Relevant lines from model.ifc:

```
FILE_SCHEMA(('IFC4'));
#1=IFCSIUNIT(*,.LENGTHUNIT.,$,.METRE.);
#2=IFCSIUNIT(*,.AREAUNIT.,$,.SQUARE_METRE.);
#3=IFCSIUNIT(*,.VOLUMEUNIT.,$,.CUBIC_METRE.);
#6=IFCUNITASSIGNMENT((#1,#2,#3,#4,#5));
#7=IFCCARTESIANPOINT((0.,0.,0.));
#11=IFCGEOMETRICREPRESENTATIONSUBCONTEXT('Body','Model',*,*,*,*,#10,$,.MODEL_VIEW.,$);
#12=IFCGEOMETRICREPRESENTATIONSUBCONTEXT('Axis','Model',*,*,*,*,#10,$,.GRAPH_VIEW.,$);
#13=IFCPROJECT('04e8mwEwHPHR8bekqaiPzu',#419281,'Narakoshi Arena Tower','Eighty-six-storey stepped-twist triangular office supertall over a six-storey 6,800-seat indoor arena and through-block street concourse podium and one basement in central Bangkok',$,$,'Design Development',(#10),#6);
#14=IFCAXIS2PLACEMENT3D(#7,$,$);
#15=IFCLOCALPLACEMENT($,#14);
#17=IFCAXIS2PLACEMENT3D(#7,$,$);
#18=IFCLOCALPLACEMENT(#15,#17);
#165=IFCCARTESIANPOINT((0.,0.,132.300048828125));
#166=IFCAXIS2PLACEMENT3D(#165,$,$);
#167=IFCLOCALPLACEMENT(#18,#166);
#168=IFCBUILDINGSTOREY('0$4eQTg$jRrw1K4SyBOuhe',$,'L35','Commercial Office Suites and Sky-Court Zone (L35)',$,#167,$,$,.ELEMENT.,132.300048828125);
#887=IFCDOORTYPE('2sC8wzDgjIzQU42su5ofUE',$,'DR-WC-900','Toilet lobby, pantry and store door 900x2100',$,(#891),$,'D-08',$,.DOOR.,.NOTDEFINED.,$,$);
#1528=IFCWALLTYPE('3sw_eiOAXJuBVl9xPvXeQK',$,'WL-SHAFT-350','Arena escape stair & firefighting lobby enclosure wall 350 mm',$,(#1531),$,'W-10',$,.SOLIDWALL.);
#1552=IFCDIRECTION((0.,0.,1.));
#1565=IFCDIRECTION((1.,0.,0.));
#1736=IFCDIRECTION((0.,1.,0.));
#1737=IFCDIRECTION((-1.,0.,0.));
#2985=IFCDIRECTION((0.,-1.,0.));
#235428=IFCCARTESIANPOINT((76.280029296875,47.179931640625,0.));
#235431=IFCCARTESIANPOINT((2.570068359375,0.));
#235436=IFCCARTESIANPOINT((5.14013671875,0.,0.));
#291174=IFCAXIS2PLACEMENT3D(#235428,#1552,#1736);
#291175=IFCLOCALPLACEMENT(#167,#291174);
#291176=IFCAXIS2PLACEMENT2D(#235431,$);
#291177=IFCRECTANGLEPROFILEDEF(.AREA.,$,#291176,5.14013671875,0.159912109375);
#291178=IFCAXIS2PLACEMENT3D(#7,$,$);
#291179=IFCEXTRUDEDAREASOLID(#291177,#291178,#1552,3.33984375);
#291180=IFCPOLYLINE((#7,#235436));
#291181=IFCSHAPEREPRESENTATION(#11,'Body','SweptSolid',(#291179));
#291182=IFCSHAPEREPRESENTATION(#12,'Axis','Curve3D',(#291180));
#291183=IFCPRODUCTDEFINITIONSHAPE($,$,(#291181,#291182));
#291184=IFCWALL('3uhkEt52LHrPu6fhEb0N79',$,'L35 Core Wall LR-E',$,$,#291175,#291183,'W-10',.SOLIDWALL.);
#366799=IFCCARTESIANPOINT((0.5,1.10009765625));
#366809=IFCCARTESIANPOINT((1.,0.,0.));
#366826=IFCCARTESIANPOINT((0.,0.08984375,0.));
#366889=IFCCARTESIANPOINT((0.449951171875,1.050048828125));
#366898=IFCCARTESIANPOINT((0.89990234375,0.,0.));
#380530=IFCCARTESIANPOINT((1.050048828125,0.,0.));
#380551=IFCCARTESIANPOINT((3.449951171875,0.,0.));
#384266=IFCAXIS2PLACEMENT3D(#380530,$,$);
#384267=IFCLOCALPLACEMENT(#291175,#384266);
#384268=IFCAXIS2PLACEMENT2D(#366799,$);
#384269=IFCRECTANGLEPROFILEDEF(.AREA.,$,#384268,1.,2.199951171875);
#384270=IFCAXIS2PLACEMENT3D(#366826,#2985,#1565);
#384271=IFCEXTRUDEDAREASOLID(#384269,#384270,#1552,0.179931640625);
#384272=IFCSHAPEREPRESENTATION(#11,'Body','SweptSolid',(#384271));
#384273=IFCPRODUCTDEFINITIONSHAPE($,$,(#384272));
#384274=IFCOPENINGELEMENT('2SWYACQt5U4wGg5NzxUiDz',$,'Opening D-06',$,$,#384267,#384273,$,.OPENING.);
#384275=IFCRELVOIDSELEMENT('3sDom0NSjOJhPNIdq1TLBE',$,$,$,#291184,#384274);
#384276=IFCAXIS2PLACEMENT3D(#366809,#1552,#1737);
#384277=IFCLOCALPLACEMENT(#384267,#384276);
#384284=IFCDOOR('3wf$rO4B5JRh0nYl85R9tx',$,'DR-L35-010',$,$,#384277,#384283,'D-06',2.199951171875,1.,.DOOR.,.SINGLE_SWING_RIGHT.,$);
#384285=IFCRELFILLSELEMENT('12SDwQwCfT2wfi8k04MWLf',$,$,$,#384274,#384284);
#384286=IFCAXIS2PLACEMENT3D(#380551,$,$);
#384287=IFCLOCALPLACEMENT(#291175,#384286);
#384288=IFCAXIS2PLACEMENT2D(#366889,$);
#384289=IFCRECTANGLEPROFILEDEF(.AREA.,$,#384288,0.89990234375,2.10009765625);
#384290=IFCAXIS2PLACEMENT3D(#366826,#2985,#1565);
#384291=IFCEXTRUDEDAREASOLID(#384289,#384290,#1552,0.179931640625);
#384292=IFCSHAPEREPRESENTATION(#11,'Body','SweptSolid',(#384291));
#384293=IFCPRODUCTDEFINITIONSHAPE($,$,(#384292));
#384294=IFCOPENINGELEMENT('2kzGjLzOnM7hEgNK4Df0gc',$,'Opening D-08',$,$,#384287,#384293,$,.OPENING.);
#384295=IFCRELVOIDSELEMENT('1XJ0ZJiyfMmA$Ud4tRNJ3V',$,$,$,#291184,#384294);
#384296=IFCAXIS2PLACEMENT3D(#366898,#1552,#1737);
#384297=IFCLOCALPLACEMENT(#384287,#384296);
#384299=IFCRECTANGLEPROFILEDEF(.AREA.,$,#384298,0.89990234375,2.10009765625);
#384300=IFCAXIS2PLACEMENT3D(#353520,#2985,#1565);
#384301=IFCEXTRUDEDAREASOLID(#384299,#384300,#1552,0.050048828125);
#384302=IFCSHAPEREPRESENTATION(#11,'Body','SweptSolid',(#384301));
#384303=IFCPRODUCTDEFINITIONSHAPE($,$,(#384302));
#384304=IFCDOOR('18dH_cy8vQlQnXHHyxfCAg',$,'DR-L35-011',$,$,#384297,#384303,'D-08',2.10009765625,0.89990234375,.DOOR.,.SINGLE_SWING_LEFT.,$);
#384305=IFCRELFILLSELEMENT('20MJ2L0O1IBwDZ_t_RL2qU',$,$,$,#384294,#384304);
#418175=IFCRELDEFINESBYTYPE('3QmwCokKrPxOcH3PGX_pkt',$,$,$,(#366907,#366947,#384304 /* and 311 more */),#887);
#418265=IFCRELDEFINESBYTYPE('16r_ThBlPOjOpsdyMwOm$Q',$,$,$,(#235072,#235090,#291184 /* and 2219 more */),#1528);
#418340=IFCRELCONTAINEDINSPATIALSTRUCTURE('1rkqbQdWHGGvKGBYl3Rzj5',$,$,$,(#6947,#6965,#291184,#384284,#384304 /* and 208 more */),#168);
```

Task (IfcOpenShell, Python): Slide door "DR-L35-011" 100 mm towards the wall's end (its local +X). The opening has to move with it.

```python
import ifcopenshell
import ifcopenshell.api.geometry
import ifcopenshell.util.placement
import ifcopenshell.util.unit

model = ifcopenshell.open("model.ifc")
unit_scale = ifcopenshell.util.unit.calculate_unit_scale(model)

door = model.by_guid("18dH_cy8vQlQnXHHyxfCAg")
opening = door.FillsVoids[0].RelatingOpeningElement
wall = opening.VoidsElements[0].RelatingBuildingElement

wall_matrix = ifcopenshell.util.placement.get_local_placement(wall.ObjectPlacement)
shift = wall_matrix[:3, 0] * 0.1 / unit_scale
before = ifcopenshell.util.placement.get_local_placement(door.ObjectPlacement)[:3, 3].copy()

# The door is placed relative to its opening, so it follows when the opening moves.
matrix = ifcopenshell.util.placement.get_local_placement(opening.ObjectPlacement)
matrix[:3, 3] += shift
ifcopenshell.api.geometry.edit_object_placement(
    model, product=opening, matrix=matrix, is_si=False, should_transform_children=True
)

after = ifcopenshell.util.placement.get_local_placement(door.ObjectPlacement)[:3, 3]
print("door moved by", (after - before).round(3) + 0.0)

model.write("model_edited.ifc")
```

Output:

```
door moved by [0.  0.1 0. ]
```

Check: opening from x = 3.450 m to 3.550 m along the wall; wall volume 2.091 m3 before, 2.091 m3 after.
